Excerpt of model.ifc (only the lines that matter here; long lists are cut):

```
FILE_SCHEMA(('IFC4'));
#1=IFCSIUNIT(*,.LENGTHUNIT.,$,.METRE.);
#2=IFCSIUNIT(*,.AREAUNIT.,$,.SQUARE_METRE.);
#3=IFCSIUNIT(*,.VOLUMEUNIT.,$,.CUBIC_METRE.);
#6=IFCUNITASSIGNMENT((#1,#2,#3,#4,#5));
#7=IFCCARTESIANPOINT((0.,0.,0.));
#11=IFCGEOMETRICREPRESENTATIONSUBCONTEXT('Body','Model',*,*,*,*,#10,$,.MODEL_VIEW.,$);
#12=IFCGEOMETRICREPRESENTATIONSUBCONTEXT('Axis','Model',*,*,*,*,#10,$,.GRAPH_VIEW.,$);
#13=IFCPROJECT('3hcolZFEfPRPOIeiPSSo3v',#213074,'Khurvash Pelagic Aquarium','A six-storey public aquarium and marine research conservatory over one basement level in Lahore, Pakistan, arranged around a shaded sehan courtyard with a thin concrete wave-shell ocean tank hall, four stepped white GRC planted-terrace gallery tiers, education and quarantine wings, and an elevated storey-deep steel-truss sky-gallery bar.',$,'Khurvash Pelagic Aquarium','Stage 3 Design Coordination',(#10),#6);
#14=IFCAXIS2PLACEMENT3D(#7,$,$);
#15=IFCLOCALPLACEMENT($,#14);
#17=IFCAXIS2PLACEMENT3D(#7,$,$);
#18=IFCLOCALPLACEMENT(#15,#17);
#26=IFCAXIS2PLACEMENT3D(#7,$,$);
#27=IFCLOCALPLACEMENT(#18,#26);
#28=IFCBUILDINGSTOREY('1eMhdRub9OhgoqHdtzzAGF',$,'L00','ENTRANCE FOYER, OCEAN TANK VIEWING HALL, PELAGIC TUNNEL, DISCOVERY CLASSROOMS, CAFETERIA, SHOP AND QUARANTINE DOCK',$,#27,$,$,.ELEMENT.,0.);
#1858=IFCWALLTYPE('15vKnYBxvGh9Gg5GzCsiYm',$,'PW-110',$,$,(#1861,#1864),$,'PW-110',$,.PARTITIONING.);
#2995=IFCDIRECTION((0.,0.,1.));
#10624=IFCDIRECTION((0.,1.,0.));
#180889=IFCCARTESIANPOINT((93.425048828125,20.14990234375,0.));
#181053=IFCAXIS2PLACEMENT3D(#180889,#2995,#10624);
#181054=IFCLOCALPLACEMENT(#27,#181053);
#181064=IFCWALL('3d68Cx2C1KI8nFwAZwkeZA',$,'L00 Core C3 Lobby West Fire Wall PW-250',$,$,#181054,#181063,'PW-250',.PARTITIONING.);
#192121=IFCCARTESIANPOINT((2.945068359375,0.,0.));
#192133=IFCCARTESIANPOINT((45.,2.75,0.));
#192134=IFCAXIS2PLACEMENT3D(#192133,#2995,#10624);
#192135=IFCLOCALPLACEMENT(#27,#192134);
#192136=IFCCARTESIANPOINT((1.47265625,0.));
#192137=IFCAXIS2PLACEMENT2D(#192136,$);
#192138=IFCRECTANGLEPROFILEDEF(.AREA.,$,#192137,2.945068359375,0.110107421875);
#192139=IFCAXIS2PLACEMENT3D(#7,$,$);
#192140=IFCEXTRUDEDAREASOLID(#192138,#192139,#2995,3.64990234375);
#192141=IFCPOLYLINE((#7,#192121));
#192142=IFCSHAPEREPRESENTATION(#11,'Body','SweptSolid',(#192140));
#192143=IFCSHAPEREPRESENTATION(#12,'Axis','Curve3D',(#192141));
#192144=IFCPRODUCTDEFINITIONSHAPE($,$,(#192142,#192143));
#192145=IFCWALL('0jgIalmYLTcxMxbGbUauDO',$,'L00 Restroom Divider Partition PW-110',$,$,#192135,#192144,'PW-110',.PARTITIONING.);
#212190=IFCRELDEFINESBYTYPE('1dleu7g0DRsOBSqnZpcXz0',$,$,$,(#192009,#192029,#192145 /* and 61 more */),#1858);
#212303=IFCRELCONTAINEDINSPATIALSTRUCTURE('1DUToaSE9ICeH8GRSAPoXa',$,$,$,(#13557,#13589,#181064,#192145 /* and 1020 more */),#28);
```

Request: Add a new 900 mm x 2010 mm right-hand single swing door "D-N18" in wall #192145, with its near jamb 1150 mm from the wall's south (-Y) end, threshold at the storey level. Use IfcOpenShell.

```python
import numpy as np
import ifcopenshell
import ifcopenshell.api.feature
import ifcopenshell.api.geometry
import ifcopenshell.api.root
import ifcopenshell.api.spatial
import ifcopenshell.geom
import ifcopenshell.util.element
import ifcopenshell.util.placement
import ifcopenshell.util.representation
import ifcopenshell.util.shape
import ifcopenshell.util.unit

model = ifcopenshell.open("model.ifc")
unit_scale = ifcopenshell.util.unit.calculate_unit_scale(model)
settings = ifcopenshell.geom.settings()


def volume(element):
    """Net volume in cubic metres, openings subtracted."""
    shape = ifcopenshell.geom.create_shape(settings, element)
    return ifcopenshell.util.shape.get_volume(shape.geometry)


wall = model.by_guid("0jgIalmYLTcxMxbGbUauDO")
storey = ifcopenshell.util.element.get_container(wall, ifc_class="IfcBuildingStorey")
context = ifcopenshell.util.representation.get_context(model, "Model", "Body", "MODEL_VIEW")
before = volume(wall)

width, height, from_end, sill = 0.9, 2.01, 1.15, 0.0  # metres

# The wall runs along its own X axis, and the end named is its -X end.
wall_shape = ifcopenshell.geom.create_shape(settings, wall)
x, y, z = ifcopenshell.util.shape.get_vertices(wall_shape.geometry).T
start = x.min() + from_end
face, thickness = float(y.min()), float(y.max() - y.min())
wall_matrix = ifcopenshell.util.placement.get_local_placement(wall.ObjectPlacement)
level = ifcopenshell.util.placement.get_local_placement(storey.ObjectPlacement)[2, 3]


def in_wall(x, y):
    """Placement at x, y metres in the wall's axes, at sill height."""
    matrix = wall_matrix.copy()
    matrix[:, 3] = wall_matrix @ np.array([x / unit_scale, y / unit_scale, 0.0, 1.0])
    matrix[2, 3] = level + sill / unit_scale
    return matrix


# Opening: a box that overshoots both wall faces by 50 mm.
opening = ifcopenshell.api.root.create_entity(model, ifc_class="IfcOpeningElement", predefined_type="OPENING")
box = ifcopenshell.api.geometry.add_wall_representation(
    model, context=context, length=width, height=height, thickness=thickness + 0.1
)
ifcopenshell.api.geometry.assign_representation(model, product=opening, representation=box)
ifcopenshell.api.geometry.edit_object_placement(model, product=opening, matrix=in_wall(start, face - 0.05), is_si=False)
ifcopenshell.api.feature.add_feature(model, feature=opening, element=wall)

door = ifcopenshell.api.root.create_entity(model, ifc_class="IfcDoor", name="D-N18", predefined_type="DOOR")
door.OverallWidth, door.OverallHeight = width / unit_scale, height / unit_scale
door.OperationType = "SINGLE_SWING_RIGHT"
body = ifcopenshell.api.geometry.add_door_representation(
    model,
    context=context,
    overall_width=door.OverallWidth,
    overall_height=door.OverallHeight,
    operation_type="SINGLE_SWING_RIGHT",
    lining_properties={"LiningDepth": thickness / unit_scale, "ThresholdDepth": thickness / unit_scale},
)
ifcopenshell.api.geometry.assign_representation(model, product=door, representation=body)
ifcopenshell.api.spatial.assign_container(model, products=[door], relating_structure=storey)
ifcopenshell.api.feature.add_filling(model, opening=opening, element=door)

# The lining spans the wall, so the door starts at the wall face.
ifcopenshell.api.geometry.edit_object_placement(model, product=door, matrix=in_wall(start, face), is_si=False)

after = volume(wall)

print(f"wall volume {before:.3f} -> {after:.3f} m3")

model.write("model-out.ifc")
```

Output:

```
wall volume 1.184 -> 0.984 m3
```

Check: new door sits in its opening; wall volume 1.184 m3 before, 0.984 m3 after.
